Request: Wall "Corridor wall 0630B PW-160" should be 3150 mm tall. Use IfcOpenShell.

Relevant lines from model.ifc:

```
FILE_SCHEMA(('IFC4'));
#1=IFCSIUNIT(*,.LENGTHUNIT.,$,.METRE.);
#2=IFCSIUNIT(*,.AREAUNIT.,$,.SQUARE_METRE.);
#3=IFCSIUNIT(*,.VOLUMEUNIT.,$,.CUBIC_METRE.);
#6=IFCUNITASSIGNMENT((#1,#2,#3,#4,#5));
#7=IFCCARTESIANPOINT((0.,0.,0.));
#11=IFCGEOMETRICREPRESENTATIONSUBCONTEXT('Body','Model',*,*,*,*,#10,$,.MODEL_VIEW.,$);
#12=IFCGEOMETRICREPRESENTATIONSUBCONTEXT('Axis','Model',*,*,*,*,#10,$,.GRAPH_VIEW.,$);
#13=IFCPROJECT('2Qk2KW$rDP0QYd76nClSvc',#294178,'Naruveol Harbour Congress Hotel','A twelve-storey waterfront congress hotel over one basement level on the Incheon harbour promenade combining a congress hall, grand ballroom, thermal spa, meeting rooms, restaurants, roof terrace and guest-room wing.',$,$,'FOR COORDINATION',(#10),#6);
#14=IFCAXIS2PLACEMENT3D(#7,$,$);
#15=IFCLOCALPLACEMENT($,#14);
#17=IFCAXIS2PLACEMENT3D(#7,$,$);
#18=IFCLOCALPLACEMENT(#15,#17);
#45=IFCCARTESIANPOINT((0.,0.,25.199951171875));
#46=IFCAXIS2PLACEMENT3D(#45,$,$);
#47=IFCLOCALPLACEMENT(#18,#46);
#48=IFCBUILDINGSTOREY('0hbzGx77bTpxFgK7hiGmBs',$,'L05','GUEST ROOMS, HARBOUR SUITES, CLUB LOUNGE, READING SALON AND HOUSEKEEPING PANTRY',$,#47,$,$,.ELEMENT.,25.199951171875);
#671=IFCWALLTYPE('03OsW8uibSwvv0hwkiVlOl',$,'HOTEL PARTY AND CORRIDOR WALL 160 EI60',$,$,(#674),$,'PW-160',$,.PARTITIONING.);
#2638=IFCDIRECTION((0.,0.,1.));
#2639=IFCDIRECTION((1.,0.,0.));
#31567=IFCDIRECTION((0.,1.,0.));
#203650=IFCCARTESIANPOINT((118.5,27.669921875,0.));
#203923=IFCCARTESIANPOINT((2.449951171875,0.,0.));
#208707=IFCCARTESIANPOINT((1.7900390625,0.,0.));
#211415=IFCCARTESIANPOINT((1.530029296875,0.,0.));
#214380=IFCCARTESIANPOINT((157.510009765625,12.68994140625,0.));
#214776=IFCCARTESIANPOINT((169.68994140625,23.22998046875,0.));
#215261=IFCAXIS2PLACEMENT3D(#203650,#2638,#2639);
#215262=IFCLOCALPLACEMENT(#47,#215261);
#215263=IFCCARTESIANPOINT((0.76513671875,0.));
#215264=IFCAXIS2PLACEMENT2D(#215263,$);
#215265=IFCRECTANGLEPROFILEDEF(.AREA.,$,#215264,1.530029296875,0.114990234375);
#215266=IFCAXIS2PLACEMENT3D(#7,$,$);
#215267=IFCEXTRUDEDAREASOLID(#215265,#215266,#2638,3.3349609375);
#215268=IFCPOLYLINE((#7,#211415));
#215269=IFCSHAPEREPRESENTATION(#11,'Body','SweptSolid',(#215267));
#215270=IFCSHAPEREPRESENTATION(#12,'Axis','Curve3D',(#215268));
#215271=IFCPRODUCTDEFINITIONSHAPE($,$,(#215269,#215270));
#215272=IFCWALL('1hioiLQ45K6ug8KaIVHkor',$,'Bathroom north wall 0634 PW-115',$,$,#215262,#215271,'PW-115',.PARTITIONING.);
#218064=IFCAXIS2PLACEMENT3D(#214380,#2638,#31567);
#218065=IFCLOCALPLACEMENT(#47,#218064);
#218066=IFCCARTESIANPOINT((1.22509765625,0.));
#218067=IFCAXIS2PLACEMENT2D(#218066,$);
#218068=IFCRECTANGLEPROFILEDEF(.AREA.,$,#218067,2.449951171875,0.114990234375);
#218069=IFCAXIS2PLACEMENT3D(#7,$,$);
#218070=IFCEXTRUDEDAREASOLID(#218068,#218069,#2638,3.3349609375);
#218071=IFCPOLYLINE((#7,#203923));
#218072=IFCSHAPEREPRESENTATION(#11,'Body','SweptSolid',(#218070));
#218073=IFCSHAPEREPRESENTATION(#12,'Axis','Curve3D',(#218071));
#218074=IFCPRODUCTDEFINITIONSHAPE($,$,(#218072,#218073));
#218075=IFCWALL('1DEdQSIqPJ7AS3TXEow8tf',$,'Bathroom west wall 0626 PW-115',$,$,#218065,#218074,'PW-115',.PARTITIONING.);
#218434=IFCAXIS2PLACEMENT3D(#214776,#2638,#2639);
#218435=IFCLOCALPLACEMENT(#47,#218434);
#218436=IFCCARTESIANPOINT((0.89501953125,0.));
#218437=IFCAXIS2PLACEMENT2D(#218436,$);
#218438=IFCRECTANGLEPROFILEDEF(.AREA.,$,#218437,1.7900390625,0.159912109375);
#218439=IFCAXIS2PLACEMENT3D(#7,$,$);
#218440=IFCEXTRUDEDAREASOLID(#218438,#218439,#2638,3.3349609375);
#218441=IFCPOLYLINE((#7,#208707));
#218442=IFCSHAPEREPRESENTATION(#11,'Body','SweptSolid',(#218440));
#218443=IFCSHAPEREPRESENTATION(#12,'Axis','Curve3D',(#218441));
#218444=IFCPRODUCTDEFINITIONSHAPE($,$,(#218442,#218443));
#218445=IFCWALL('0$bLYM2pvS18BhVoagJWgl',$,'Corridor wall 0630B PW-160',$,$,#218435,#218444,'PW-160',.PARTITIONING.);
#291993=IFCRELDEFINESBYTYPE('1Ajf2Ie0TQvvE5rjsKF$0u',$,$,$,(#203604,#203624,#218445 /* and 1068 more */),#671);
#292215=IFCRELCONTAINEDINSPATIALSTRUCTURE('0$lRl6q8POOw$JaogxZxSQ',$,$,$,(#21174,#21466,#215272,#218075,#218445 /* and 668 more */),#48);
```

```python
import ifcopenshell
import ifcopenshell.geom
import ifcopenshell.util.representation
import ifcopenshell.util.shape
import ifcopenshell.util.unit

model = ifcopenshell.open("model.ifc")
unit_scale = ifcopenshell.util.unit.calculate_unit_scale(model)
settings = ifcopenshell.geom.settings()


def volume(element):
    """Net volume in cubic metres, openings subtracted."""
    shape = ifcopenshell.geom.create_shape(settings, element)
    return ifcopenshell.util.shape.get_volume(shape.geometry)


wall = model.by_guid("0$bLYM2pvS18BhVoagJWgl")
before = volume(wall)

body = ifcopenshell.util.representation.get_representation(wall, "Model", "Body")
solid = body.Items[0]
old_height = solid.Depth
solid.Depth = 3.15 / unit_scale
after = volume(wall)

print(f"height {old_height:g} -> {solid.Depth:g}, volume {before:.3f} -> {after:.3f} m3")

model.write("model_rev.ifc")
```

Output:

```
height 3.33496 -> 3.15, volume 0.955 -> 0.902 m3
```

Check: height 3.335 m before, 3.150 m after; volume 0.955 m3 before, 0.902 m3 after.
